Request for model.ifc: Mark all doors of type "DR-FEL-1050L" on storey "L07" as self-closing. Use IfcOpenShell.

First a look at what the model holds.

```python
import ifcopenshell
import ifcopenshell.util.element

model = ifcopenshell.open("model.ifc")
print(model.schema)
storey = next(s for s in model.by_type("IfcBuildingStorey") if s.Name == "L07")
doors = [e for e in ifcopenshell.util.element.get_decomposition(storey) if e.is_a("IfcDoor")]
seen = {}
for e in doors:
    element_type = ifcopenshell.util.element.get_type(e)
    key = (element_type.Name if element_type != e and element_type else None, ifcopenshell.util.element.get_pset(e, "Pset_DoorCommon", "SelfClosing"))
    seen[key] = seen.get(key, 0) + 1
for (name, value), count in sorted(seen.items(), key=str):
    print(count, "x", name, "|", value)
```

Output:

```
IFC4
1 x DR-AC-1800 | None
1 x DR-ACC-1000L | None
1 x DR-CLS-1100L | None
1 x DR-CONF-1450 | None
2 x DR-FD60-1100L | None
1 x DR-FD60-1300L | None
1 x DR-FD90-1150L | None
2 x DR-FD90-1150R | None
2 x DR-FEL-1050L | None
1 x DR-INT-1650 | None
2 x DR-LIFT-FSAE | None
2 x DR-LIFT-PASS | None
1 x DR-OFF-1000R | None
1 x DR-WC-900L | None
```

```python
import ifcopenshell
import ifcopenshell.api.pset
import ifcopenshell.util.element

model = ifcopenshell.open("model.ifc")

storey = next(s for s in model.by_type("IfcBuildingStorey") if s.Name == "L07")
doors = [e for e in ifcopenshell.util.element.get_decomposition(storey) if e.is_a("IfcDoor")]

count = 0
for e in doors:
    element_type = ifcopenshell.util.element.get_type(e)
    if element_type in (None, e) or element_type.Name != "DR-FEL-1050L":
        continue
    # add_pset returns the element's existing set when there is one.
    pset = ifcopenshell.api.pset.add_pset(model, product=e, name="Pset_DoorCommon")
    ifcopenshell.api.pset.edit_pset(model, pset=pset, properties={"SelfClosing": True})
    count += 1

print(count, "doors updated")

model.write("model_rev.ifc")
```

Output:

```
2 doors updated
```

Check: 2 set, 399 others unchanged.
